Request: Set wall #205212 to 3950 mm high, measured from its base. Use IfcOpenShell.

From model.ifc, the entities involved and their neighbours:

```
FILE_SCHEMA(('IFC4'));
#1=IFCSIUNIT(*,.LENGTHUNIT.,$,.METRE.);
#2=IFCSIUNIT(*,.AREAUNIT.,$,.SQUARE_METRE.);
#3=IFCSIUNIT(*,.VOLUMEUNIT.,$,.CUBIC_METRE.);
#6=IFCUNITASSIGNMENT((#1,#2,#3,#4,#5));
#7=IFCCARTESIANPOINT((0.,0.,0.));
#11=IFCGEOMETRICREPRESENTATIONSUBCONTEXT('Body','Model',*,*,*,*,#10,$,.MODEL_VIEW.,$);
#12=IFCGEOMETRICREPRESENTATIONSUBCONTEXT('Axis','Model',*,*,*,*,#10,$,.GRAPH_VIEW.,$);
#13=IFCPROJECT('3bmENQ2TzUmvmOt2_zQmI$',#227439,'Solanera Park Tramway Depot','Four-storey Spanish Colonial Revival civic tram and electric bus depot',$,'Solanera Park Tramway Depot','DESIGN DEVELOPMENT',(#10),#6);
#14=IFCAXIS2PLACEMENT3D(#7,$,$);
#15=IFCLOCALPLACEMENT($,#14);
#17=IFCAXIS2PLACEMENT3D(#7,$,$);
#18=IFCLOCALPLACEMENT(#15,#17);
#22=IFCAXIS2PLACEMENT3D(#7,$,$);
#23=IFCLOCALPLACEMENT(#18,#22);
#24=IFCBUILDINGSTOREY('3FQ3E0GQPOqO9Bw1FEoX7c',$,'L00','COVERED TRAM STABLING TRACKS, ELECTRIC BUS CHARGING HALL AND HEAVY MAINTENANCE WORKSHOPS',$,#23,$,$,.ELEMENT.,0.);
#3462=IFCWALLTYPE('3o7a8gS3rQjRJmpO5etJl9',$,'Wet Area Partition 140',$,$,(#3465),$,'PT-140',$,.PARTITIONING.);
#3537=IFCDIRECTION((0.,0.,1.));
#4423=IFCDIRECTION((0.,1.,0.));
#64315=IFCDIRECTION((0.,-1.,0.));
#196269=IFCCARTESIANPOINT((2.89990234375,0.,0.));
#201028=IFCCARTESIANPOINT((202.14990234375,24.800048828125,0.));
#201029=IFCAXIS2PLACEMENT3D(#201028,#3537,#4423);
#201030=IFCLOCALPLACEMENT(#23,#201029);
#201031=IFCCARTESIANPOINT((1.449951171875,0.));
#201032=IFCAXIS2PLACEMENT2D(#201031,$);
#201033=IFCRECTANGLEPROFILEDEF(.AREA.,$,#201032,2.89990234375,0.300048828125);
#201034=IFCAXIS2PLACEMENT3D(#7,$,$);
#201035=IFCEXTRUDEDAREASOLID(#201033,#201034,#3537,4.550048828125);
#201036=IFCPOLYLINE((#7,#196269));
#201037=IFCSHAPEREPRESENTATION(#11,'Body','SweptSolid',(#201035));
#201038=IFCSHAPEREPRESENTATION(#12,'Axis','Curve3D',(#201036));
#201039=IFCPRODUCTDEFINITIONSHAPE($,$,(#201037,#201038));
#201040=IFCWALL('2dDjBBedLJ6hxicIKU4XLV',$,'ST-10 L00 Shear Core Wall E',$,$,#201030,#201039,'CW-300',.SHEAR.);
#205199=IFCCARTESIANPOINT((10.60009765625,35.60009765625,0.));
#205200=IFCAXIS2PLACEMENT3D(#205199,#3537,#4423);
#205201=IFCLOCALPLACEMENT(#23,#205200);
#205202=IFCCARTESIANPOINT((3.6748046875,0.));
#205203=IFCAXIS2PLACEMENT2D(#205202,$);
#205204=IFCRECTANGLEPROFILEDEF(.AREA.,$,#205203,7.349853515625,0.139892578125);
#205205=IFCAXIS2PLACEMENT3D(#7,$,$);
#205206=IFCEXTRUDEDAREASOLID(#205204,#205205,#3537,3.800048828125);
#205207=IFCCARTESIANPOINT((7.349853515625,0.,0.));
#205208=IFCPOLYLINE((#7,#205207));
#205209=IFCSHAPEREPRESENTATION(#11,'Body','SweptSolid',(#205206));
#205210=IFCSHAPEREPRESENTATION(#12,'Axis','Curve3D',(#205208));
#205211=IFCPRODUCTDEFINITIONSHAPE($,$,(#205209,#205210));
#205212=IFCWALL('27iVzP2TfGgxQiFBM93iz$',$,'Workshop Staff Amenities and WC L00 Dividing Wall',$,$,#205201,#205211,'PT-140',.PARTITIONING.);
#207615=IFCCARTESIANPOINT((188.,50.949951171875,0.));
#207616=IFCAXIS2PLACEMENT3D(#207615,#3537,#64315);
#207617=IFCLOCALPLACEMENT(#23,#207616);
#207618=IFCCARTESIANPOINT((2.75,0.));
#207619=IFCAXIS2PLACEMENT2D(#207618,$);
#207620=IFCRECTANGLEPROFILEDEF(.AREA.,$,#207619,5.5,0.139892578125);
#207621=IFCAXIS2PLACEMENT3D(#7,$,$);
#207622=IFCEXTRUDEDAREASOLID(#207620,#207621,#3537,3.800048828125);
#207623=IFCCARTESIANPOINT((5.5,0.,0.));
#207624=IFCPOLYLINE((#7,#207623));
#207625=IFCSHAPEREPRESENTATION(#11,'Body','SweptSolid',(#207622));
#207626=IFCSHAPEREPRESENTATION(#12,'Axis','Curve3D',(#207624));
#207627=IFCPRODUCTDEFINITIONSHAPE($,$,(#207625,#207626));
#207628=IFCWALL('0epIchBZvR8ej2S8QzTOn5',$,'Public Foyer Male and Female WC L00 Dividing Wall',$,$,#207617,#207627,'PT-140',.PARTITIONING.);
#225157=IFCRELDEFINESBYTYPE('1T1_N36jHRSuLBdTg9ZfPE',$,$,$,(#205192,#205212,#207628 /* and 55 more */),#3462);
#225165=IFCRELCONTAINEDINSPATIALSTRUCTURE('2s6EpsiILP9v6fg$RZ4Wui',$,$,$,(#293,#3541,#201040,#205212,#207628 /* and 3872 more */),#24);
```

```python
import ifcopenshell
import ifcopenshell.geom
import ifcopenshell.util.representation
import ifcopenshell.util.shape
import ifcopenshell.util.unit

model = ifcopenshell.open("model.ifc")
unit_scale = ifcopenshell.util.unit.calculate_unit_scale(model)
settings = ifcopenshell.geom.settings()


def volume(element):
    """Net volume in cubic metres, openings subtracted."""
    shape = ifcopenshell.geom.create_shape(settings, element)
    return ifcopenshell.util.shape.get_volume(shape.geometry)


wall = model.by_id(205212)
before = volume(wall)

body = ifcopenshell.util.representation.get_representation(wall, "Model", "Body")
solid = body.Items[0]
old_height = solid.Depth
solid.Depth = 3.95 / unit_scale
after = volume(wall)

print(f"height {old_height:g} -> {solid.Depth:g}, volume {before:.3f} -> {after:.3f} m3")

model.write("model_v2.ifc")
```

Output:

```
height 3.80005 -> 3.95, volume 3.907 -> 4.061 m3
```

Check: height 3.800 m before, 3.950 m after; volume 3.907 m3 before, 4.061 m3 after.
